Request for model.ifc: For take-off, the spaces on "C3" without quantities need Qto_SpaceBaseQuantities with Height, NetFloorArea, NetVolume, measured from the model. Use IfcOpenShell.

First a look at what the model holds.

```python
import ifcopenshell
import ifcopenshell.util.element
import ifcopenshell.util.unit

model = ifcopenshell.open("model.ifc")
print(model.schema)
for unit_type in ("LENGTHUNIT", "AREAUNIT", "VOLUMEUNIT"):
    print(unit_type, ifcopenshell.util.unit.calculate_unit_scale(model, unit_type))
storey = next(s for s in model.by_type("IfcBuildingStorey") if s.Name == "C3")
spaces = [e for e in ifcopenshell.util.element.get_decomposition(storey) if e.is_a("IfcSpace")]
for e in sorted(spaces, key=lambda e: e.id()):
    print(e.id(), e.is_a(), e.Name, list(ifcopenshell.util.element.get_psets(e, qtos_only=True)), sep=" | ")
```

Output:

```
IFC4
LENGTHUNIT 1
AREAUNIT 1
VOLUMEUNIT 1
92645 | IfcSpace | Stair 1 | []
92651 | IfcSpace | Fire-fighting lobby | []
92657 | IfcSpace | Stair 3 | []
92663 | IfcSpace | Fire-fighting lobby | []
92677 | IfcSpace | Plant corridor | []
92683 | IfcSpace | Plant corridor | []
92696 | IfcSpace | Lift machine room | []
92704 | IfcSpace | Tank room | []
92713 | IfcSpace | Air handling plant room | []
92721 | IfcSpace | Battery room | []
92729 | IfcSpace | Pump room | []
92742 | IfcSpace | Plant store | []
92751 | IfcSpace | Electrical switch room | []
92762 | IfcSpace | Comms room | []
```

```python
import ifcopenshell
import ifcopenshell.api.pset
import ifcopenshell.geom
import ifcopenshell.util.element
import ifcopenshell.util.shape
import ifcopenshell.util.unit

model = ifcopenshell.open("model.ifc")
unit_scale = ifcopenshell.util.unit.calculate_unit_scale(model)
area_scale = ifcopenshell.util.unit.calculate_unit_scale(model, "AREAUNIT")
volume_scale = ifcopenshell.util.unit.calculate_unit_scale(model, "VOLUMEUNIT")
settings = ifcopenshell.geom.settings()

storey = next(s for s in model.by_type("IfcBuildingStorey") if s.Name == "C3")
spaces = [e for e in ifcopenshell.util.element.get_decomposition(storey) if e.is_a("IfcSpace")]

for e in sorted(spaces, key=lambda e: e.id()):
    if ifcopenshell.util.element.get_psets(e, qtos_only=True, should_inherit=False):
        continue
    # Geometry comes back in metres, in the element's own axes.
    shape = ifcopenshell.geom.create_shape(settings, e)
    values = {
        "Height": ifcopenshell.util.shape.get_z(shape.geometry) / unit_scale,
        "NetFloorArea": ifcopenshell.util.shape.get_footprint_area(shape.geometry) / area_scale,
        "NetVolume": ifcopenshell.util.shape.get_volume(shape.geometry) / volume_scale,
    }
    qto = ifcopenshell.api.pset.add_qto(model, product=e, name="Qto_SpaceBaseQuantities")
    ifcopenshell.api.pset.edit_qto(model, qto=qto, properties=values)
    print(e.id(), {k: round(v, 3) for k, v in values.items()})

model.write("model_v2.ifc")
```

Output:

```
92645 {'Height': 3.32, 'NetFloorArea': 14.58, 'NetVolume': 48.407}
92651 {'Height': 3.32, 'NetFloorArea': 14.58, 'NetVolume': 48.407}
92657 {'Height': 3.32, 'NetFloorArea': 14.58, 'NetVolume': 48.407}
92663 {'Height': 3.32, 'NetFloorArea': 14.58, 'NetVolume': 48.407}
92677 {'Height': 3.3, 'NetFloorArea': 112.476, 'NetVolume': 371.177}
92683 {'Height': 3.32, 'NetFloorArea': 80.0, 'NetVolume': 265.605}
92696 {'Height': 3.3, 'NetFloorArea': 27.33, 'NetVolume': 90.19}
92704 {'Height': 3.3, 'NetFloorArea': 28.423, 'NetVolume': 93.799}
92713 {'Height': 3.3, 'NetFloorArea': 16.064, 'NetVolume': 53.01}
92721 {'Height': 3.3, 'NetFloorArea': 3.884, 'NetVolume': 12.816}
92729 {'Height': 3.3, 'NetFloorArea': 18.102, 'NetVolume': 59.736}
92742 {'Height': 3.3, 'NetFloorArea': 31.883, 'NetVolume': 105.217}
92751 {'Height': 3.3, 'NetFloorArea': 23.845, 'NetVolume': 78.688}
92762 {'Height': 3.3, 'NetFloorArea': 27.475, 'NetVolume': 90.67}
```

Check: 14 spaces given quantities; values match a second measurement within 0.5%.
